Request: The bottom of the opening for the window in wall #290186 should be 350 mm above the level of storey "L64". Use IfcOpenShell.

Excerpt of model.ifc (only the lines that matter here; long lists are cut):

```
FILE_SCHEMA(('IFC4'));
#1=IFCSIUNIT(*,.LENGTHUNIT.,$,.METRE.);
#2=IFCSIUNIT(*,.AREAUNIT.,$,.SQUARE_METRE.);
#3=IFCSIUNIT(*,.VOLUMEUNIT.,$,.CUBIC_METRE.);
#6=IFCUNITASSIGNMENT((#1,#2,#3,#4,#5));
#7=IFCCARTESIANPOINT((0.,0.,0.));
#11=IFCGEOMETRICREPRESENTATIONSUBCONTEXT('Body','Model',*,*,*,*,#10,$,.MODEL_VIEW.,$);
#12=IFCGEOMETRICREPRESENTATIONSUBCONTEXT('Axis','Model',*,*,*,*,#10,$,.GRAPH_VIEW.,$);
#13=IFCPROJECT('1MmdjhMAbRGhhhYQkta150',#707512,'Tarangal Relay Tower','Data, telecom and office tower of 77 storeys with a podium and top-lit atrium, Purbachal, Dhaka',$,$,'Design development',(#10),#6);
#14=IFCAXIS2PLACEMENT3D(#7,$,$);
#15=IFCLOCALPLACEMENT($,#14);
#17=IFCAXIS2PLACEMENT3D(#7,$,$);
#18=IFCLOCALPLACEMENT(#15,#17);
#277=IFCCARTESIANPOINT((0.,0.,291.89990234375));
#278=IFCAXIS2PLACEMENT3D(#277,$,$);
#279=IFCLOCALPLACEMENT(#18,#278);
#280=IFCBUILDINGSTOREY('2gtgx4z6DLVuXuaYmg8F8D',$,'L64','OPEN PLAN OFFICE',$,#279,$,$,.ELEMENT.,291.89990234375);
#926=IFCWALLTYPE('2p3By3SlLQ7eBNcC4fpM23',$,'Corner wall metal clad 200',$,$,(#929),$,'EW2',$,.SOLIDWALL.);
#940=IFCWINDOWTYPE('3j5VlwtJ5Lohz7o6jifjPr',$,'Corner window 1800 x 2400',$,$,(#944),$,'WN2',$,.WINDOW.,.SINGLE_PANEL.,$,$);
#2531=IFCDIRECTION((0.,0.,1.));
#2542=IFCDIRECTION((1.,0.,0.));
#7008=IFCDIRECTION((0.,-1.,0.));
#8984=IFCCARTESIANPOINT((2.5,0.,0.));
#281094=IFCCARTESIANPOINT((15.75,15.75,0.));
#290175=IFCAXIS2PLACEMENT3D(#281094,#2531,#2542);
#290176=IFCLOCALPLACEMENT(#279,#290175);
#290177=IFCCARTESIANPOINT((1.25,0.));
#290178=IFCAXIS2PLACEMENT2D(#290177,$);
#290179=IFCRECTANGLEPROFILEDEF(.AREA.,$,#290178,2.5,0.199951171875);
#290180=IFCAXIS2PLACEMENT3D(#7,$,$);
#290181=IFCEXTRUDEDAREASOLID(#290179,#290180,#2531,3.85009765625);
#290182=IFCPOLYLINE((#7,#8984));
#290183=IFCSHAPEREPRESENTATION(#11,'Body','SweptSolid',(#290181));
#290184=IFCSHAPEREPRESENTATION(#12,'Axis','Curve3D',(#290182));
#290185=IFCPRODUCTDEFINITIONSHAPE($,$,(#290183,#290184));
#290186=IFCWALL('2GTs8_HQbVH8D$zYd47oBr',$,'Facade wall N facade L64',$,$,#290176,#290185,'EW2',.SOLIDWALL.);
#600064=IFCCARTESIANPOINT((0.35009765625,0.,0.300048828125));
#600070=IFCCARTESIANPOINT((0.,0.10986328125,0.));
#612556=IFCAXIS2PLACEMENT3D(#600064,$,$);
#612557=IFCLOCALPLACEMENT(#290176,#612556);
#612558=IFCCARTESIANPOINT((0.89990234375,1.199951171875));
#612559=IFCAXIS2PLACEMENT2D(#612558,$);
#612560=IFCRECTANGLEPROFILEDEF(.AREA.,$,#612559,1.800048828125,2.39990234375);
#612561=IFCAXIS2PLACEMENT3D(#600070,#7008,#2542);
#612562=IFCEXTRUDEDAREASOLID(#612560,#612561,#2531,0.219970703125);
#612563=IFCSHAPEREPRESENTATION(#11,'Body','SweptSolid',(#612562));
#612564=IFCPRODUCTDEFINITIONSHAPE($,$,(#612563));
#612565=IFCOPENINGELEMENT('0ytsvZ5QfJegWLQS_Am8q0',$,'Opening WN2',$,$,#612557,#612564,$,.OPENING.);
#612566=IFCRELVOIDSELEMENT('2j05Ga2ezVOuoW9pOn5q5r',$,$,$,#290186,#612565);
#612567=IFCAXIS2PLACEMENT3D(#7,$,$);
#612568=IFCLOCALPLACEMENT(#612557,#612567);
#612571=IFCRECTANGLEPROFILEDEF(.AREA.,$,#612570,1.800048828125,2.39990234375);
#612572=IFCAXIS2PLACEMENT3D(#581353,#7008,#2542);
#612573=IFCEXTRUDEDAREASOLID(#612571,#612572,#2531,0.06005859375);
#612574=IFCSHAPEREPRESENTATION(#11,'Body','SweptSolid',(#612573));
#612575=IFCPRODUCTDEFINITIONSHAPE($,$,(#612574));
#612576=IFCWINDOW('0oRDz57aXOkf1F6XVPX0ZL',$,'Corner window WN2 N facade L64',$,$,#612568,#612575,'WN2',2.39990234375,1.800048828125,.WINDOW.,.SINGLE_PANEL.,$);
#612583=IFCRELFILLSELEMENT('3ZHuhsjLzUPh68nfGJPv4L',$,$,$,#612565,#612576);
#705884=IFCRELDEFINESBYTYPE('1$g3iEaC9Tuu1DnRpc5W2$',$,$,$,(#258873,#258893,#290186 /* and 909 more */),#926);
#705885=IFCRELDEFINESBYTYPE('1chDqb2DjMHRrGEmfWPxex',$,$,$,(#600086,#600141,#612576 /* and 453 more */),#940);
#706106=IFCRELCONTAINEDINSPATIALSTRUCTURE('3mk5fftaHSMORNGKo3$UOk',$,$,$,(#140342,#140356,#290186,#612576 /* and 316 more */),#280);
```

```python
import numpy as np
import ifcopenshell
import ifcopenshell.api.geometry
import ifcopenshell.geom
import ifcopenshell.util.element
import ifcopenshell.util.placement
import ifcopenshell.util.shape
import ifcopenshell.util.unit

model = ifcopenshell.open("model.ifc")
unit_scale = ifcopenshell.util.unit.calculate_unit_scale(model)

window = model.by_guid("0oRDz57aXOkf1F6XVPX0ZL")
opening = window.FillsVoids[0].RelatingOpeningElement
storey = ifcopenshell.util.element.get_container(window, ifc_class="IfcBuildingStorey")
level = ifcopenshell.util.placement.get_local_placement(storey.ObjectPlacement)[2, 3]

# The opening's origin need not be at the sill, so measure its lowest point.
shape = ifcopenshell.geom.create_shape(ifcopenshell.geom.settings(), opening)
bottom = ifcopenshell.util.shape.get_shape_bottom_elevation(shape, shape.geometry) / unit_scale
dz = level + 0.35 / unit_scale - bottom

shift = np.array([0.0, 0.0, dz])
# The window is placed relative to its opening, so it follows when the opening moves.
matrix = ifcopenshell.util.placement.get_local_placement(opening.ObjectPlacement)
matrix[:3, 3] += shift
ifcopenshell.api.geometry.edit_object_placement(
    model, product=opening, matrix=matrix, is_si=False, should_transform_children=True
)

print(f"moved by {dz * unit_scale:+.3f} m")

model.write("model_rev.ifc")
```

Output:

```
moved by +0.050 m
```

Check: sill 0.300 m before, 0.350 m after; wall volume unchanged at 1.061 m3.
